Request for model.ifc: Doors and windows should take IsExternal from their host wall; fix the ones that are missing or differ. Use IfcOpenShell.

First a look at what the model holds.

```python
import ifcopenshell
import ifcopenshell.util.element

model = ifcopenshell.open("model.ifc")
print(model.schema)
seen = {}
for e in model.by_type("IfcDoor") + model.by_type("IfcWindow"):
    if not e.FillsVoids:
        continue
    host = e.FillsVoids[0].RelatingOpeningElement.VoidsElements[0].RelatingBuildingElement
    own = ifcopenshell.util.element.get_pset(e, f"Pset_{e.is_a()[3:].removesuffix('StandardCase')}Common", "IsExternal")
    wall = ifcopenshell.util.element.get_pset(host, "Pset_WallCommon", "IsExternal")
    seen[e.is_a(), own, wall] = seen.get((e.is_a(), own, wall), 0) + 1
for (cls, own, wall), count in sorted(seen.items(), key=str):
    print(count, cls, "IsExternal:", own, "| host wall:", wall)
```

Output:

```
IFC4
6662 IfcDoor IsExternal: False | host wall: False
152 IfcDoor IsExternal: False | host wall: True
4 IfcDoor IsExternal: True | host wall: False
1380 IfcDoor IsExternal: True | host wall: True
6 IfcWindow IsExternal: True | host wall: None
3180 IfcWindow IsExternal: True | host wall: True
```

```python
import ifcopenshell
import ifcopenshell.api.pset
import ifcopenshell.util.element

model = ifcopenshell.open("model.ifc")

count = 0
for ifc_class, pset_name in (("IfcDoor", "Pset_DoorCommon"), ("IfcWindow", "Pset_WindowCommon")):
    for e in model.by_type(ifc_class):
        if not e.FillsVoids:
            continue
        host = e.FillsVoids[0].RelatingOpeningElement.VoidsElements[0].RelatingBuildingElement
        external = ifcopenshell.util.element.get_pset(host, "Pset_WallCommon", "IsExternal")
        if external is None or ifcopenshell.util.element.get_pset(e, pset_name, "IsExternal") == external:
            continue
        pset = ifcopenshell.api.pset.add_pset(model, product=e, name=pset_name)
        ifcopenshell.api.pset.edit_pset(model, pset=pset, properties={"IsExternal": external})
        count += 1

print(count, "updated")

model.write("model_v2.ifc")
```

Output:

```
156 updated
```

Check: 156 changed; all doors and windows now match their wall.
